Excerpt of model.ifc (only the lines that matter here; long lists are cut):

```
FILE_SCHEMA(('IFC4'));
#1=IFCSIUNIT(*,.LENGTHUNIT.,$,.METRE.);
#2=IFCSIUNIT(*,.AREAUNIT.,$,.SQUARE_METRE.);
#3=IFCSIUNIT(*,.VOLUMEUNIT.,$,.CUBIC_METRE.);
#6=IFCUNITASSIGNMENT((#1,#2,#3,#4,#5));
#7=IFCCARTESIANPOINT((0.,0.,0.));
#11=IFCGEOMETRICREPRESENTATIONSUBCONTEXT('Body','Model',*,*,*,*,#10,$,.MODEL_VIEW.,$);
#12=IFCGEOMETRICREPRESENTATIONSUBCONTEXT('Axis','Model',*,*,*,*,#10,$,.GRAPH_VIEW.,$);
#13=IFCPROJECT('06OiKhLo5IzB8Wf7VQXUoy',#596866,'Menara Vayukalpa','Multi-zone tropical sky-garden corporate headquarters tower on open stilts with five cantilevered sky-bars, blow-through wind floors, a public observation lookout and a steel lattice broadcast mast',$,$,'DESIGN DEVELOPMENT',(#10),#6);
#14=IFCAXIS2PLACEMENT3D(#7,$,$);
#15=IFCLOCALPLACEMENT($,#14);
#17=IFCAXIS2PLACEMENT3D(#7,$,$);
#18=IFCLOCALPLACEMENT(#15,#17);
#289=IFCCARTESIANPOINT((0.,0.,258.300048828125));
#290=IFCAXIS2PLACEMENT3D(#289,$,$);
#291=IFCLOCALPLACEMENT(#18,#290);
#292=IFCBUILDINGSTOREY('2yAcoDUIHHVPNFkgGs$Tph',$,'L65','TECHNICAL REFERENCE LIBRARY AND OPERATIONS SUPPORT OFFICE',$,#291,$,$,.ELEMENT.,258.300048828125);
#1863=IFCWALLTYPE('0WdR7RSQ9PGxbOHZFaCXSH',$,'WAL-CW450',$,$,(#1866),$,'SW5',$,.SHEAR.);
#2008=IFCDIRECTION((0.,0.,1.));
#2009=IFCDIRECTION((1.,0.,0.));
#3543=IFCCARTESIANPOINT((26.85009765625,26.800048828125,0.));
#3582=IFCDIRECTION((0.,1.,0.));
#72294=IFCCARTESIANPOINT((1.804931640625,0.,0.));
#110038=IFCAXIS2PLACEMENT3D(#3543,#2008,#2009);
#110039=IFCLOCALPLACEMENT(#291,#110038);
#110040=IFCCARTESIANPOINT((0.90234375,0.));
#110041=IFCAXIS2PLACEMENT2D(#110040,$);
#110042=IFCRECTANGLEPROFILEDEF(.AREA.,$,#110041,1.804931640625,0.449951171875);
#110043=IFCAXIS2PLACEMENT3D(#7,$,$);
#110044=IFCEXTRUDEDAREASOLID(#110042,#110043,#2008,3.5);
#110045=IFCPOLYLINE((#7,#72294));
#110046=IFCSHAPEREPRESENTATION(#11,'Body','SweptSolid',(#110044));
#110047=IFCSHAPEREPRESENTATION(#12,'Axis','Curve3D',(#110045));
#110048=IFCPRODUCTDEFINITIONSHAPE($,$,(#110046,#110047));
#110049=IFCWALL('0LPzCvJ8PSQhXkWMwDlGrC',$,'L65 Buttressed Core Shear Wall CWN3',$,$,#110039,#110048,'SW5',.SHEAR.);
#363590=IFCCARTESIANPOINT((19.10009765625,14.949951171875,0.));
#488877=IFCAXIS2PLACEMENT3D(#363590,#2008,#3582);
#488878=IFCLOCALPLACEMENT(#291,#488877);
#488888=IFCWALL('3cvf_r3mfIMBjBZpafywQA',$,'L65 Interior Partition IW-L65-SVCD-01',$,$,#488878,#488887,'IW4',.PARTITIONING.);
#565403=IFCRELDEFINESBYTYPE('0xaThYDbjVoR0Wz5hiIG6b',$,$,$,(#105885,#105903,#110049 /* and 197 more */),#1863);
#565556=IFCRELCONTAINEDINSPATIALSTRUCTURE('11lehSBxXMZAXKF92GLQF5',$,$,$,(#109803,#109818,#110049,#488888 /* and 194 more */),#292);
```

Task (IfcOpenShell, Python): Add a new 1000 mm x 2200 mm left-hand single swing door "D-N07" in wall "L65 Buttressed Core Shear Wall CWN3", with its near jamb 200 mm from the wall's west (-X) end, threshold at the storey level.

```python
import numpy as np
import ifcopenshell
import ifcopenshell.api.feature
import ifcopenshell.api.geometry
import ifcopenshell.api.root
import ifcopenshell.api.spatial
import ifcopenshell.geom
import ifcopenshell.util.element
import ifcopenshell.util.placement
import ifcopenshell.util.representation
import ifcopenshell.util.shape
import ifcopenshell.util.unit

model = ifcopenshell.open("model.ifc")
unit_scale = ifcopenshell.util.unit.calculate_unit_scale(model)
settings = ifcopenshell.geom.settings()


def volume(element):
    """Net volume in cubic metres, openings subtracted."""
    shape = ifcopenshell.geom.create_shape(settings, element)
    return ifcopenshell.util.shape.get_volume(shape.geometry)


wall = model.by_guid("0LPzCvJ8PSQhXkWMwDlGrC")
storey = ifcopenshell.util.element.get_container(wall, ifc_class="IfcBuildingStorey")
context = ifcopenshell.util.representation.get_context(model, "Model", "Body", "MODEL_VIEW")
before = volume(wall)

width, height, from_end, sill = 1, 2.2, 0.2, 0.0  # metres

# The wall runs along its own X axis, and the end named is its -X end.
wall_shape = ifcopenshell.geom.create_shape(settings, wall)
x, y, z = ifcopenshell.util.shape.get_vertices(wall_shape.geometry).T
start = x.min() + from_end
face, thickness = float(y.min()), float(y.max() - y.min())
wall_matrix = ifcopenshell.util.placement.get_local_placement(wall.ObjectPlacement)
level = ifcopenshell.util.placement.get_local_placement(storey.ObjectPlacement)[2, 3]


def in_wall(x, y):
    """Placement at x, y metres in the wall's axes, at sill height."""
    matrix = wall_matrix.copy()
    matrix[:, 3] = wall_matrix @ np.array([x / unit_scale, y / unit_scale, 0.0, 1.0])
    matrix[2, 3] = level + sill / unit_scale
    return matrix


# Opening: a box that overshoots both wall faces by 50 mm.
opening = ifcopenshell.api.root.create_entity(model, ifc_class="IfcOpeningElement", predefined_type="OPENING")
box = ifcopenshell.api.geometry.add_wall_representation(
    model, context=context, length=width, height=height, thickness=thickness + 0.1
)
ifcopenshell.api.geometry.assign_representation(model, product=opening, representation=box)
ifcopenshell.api.geometry.edit_object_placement(model, product=opening, matrix=in_wall(start, face - 0.05), is_si=False)
ifcopenshell.api.feature.add_feature(model, feature=opening, element=wall)

door = ifcopenshell.api.root.create_entity(model, ifc_class="IfcDoor", name="D-N07", predefined_type="DOOR")
door.OverallWidth, door.OverallHeight = width / unit_scale, height / unit_scale
door.OperationType = "SINGLE_SWING_LEFT"
body = ifcopenshell.api.geometry.add_door_representation(
    model,
    context=context,
    overall_width=door.OverallWidth,
    overall_height=door.OverallHeight,
    operation_type="SINGLE_SWING_LEFT",
    lining_properties={"LiningDepth": thickness / unit_scale, "ThresholdDepth": thickness / unit_scale},
)
ifcopenshell.api.geometry.assign_representation(model, product=door, representation=body)
ifcopenshell.api.spatial.assign_container(model, products=[door], relating_structure=storey)
ifcopenshell.api.feature.add_filling(model, opening=opening, element=door)

# The lining spans the wall, so the door starts at the wall face.
ifcopenshell.api.geometry.edit_object_placement(model, product=door, matrix=in_wall(start, face), is_si=False)

after = volume(wall)

print(f"wall volume {before:.3f} -> {after:.3f} m3")

model.write("model_rev.ifc")
```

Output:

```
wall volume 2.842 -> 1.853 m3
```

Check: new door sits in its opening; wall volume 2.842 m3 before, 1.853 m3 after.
